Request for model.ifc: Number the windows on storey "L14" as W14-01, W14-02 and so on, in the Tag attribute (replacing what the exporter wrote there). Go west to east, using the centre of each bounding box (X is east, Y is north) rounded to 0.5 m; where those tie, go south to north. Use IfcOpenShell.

First a look at what the model holds.

```python
import ifcopenshell
import ifcopenshell.util.element
import ifcopenshell.util.placement

model = ifcopenshell.open("model.ifc")
print(model.schema)
storey = next(s for s in model.by_type("IfcBuildingStorey") if s.Name == "L14")
windows = [e for e in ifcopenshell.util.element.get_decomposition(storey) if e.is_a("IfcWindow")]
for e in sorted(windows, key=lambda e: e.id()):
    origin = ifcopenshell.util.placement.get_local_placement(e.ObjectPlacement)[:3, 3]
    print(e.id(), e.Tag, e.Name, origin.round(2) + 0.0, sep=" | ")
```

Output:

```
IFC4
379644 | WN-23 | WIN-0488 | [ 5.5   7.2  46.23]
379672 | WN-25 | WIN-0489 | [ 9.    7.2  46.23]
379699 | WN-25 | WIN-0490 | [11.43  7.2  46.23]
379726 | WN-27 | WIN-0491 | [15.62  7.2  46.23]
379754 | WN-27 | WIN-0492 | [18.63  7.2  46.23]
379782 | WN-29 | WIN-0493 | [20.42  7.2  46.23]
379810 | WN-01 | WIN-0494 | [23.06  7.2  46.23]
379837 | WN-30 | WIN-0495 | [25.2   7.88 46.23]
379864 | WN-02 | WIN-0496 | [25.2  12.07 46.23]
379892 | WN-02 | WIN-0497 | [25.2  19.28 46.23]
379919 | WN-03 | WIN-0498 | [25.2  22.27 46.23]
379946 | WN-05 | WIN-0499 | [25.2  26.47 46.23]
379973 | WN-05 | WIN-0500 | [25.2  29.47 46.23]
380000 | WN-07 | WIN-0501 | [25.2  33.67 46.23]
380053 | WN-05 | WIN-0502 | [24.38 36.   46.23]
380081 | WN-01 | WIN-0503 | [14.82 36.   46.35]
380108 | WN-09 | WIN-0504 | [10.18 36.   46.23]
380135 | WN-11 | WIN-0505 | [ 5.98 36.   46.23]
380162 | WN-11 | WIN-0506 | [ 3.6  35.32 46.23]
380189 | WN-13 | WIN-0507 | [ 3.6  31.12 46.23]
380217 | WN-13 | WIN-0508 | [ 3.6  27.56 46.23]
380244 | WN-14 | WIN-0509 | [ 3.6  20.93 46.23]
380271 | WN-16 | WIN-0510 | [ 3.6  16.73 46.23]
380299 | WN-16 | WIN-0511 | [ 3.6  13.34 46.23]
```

```python
import ifcopenshell
import ifcopenshell.geom
import ifcopenshell.util.element
import ifcopenshell.util.shape

model = ifcopenshell.open("model.ifc")
settings = ifcopenshell.geom.settings()
settings.set("use-world-coords", True)


def centre(element):
    shape = ifcopenshell.geom.create_shape(settings, element)
    return ifcopenshell.util.shape.get_bbox_centroid(shape.geometry)


storey = next(s for s in model.by_type("IfcBuildingStorey") if s.Name == "L14")
windows = [e for e in ifcopenshell.util.element.get_decomposition(storey) if e.is_a("IfcWindow")]

# Insertion points can sit at a corner or the storey origin, so sort by the geometry (in metres).
centres = {e: centre(e) for e in windows}
windows.sort(key=lambda e: (round(centres[e][0] / 0.5), centres[e][1]))

for i, e in enumerate(windows, start=1):
    number = f"W14-{i:02d}"
    e.Tag = number
    print(e.id(), number)

model.write("model_edited.ifc")
```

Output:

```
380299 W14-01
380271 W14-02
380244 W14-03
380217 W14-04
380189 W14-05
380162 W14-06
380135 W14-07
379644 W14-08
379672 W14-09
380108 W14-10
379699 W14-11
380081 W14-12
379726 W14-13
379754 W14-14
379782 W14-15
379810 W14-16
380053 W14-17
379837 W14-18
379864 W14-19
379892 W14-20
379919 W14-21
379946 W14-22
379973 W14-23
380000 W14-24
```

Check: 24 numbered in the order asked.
